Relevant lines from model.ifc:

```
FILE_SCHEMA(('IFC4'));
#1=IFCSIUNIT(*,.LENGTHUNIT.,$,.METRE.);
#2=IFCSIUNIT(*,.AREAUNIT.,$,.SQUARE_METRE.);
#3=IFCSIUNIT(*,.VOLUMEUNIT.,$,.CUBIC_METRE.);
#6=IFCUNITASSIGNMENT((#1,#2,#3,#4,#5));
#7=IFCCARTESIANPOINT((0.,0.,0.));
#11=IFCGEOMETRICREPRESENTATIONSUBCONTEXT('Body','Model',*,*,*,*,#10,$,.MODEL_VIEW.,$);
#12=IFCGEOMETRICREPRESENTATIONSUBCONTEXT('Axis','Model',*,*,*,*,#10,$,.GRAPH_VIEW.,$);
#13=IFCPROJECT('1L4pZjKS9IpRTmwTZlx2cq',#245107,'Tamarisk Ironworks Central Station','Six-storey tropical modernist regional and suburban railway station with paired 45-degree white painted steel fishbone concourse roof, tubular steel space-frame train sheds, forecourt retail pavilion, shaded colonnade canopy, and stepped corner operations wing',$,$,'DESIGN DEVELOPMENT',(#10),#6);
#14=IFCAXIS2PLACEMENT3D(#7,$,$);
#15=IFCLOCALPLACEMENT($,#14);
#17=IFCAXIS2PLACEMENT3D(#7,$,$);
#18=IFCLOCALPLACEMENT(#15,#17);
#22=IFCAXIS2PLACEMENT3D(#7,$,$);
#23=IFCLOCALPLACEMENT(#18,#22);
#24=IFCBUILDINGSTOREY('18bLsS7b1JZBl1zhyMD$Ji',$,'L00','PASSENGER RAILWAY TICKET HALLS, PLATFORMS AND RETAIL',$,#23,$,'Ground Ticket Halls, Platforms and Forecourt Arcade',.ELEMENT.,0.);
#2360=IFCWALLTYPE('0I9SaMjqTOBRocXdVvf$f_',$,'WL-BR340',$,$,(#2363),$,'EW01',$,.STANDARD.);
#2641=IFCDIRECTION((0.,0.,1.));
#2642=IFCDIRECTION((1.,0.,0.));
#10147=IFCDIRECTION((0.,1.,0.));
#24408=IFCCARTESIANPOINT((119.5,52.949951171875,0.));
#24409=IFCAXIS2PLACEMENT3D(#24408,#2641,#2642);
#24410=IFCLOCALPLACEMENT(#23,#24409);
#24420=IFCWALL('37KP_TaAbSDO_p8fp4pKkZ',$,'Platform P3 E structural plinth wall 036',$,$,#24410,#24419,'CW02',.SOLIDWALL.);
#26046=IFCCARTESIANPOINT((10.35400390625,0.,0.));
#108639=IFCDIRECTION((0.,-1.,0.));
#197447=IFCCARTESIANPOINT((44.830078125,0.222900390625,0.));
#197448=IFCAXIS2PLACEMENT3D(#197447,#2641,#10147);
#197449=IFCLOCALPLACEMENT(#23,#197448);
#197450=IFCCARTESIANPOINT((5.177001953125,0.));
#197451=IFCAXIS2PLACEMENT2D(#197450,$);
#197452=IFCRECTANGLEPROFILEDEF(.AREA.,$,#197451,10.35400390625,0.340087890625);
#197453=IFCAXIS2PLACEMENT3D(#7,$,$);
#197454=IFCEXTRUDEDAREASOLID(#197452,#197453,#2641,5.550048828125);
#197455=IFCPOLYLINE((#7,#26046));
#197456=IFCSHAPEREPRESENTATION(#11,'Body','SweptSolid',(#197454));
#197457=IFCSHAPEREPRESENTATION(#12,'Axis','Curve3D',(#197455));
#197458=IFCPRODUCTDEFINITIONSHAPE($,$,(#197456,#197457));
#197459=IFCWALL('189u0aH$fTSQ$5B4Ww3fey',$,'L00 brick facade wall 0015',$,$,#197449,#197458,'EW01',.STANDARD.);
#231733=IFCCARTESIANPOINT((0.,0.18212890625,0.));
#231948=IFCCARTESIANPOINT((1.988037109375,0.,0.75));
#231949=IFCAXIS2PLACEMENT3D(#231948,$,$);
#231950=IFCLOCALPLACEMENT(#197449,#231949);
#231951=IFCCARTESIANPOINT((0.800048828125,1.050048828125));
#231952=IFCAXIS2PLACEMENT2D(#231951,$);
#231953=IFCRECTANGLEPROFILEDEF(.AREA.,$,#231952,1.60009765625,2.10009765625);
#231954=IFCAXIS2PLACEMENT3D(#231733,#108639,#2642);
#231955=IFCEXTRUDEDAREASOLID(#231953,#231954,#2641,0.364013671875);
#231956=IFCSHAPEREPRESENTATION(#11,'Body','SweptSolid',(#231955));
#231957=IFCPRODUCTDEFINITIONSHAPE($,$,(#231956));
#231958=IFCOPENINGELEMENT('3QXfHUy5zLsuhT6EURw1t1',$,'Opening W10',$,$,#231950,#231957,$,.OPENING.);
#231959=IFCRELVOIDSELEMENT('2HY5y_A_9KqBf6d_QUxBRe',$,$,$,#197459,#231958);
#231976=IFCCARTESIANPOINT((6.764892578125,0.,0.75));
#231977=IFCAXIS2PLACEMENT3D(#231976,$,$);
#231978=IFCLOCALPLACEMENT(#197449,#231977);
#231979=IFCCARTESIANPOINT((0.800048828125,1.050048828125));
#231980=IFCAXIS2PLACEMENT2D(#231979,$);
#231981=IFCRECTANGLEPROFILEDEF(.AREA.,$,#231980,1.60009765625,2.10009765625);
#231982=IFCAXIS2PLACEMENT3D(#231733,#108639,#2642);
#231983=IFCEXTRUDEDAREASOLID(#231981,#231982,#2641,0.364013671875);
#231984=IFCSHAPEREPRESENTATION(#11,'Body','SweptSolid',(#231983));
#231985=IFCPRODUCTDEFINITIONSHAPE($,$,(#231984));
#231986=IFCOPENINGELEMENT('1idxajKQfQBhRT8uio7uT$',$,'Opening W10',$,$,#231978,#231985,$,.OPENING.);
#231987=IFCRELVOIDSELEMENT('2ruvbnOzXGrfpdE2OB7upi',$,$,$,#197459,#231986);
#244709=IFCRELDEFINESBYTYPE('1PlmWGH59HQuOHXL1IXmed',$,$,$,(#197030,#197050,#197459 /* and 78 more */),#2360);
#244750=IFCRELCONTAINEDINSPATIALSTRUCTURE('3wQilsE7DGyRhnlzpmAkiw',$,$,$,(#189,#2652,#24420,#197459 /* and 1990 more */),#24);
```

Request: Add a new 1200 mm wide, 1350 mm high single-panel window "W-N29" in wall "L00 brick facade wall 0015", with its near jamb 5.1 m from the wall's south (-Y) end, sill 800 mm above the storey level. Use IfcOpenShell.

```python
import numpy as np
import ifcopenshell
import ifcopenshell.api.feature
import ifcopenshell.api.geometry
import ifcopenshell.api.root
import ifcopenshell.api.spatial
import ifcopenshell.geom
import ifcopenshell.util.element
import ifcopenshell.util.placement
import ifcopenshell.util.representation
import ifcopenshell.util.shape
import ifcopenshell.util.unit

model = ifcopenshell.open("model.ifc")
unit_scale = ifcopenshell.util.unit.calculate_unit_scale(model)
settings = ifcopenshell.geom.settings()


def volume(element):
    """Net volume in cubic metres, openings subtracted."""
    shape = ifcopenshell.geom.create_shape(settings, element)
    return ifcopenshell.util.shape.get_volume(shape.geometry)


wall = model.by_guid("189u0aH$fTSQ$5B4Ww3fey")
storey = ifcopenshell.util.element.get_container(wall, ifc_class="IfcBuildingStorey")
context = ifcopenshell.util.representation.get_context(model, "Model", "Body", "MODEL_VIEW")
before = volume(wall)

width, height, from_end, sill = 1.2, 1.35, 5.1, 0.8  # metres

# The wall runs along its own X axis, and the end named is its -X end.
wall_shape = ifcopenshell.geom.create_shape(settings, wall)
x, y, z = ifcopenshell.util.shape.get_vertices(wall_shape.geometry).T
start = x.min() + from_end
face, thickness = float(y.min()), float(y.max() - y.min())
wall_matrix = ifcopenshell.util.placement.get_local_placement(wall.ObjectPlacement)
level = ifcopenshell.util.placement.get_local_placement(storey.ObjectPlacement)[2, 3]


def in_wall(x, y):
    """Placement at x, y metres in the wall's axes, at sill height."""
    matrix = wall_matrix.copy()
    matrix[:, 3] = wall_matrix @ np.array([x / unit_scale, y / unit_scale, 0.0, 1.0])
    matrix[2, 3] = level + sill / unit_scale
    return matrix


# Opening: a box that overshoots both wall faces by 50 mm.
opening = ifcopenshell.api.root.create_entity(model, ifc_class="IfcOpeningElement", predefined_type="OPENING")
box = ifcopenshell.api.geometry.add_wall_representation(
    model, context=context, length=width, height=height, thickness=thickness + 0.1
)
ifcopenshell.api.geometry.assign_representation(model, product=opening, representation=box)
ifcopenshell.api.geometry.edit_object_placement(model, product=opening, matrix=in_wall(start, face - 0.05), is_si=False)
ifcopenshell.api.feature.add_feature(model, feature=opening, element=wall)

window = ifcopenshell.api.root.create_entity(model, ifc_class="IfcWindow", name="W-N29", predefined_type="WINDOW")
window.OverallWidth, window.OverallHeight = width / unit_scale, height / unit_scale
window.PartitioningType = "SINGLE_PANEL"
body = ifcopenshell.api.geometry.add_window_representation(
    model,
    context=context,
    overall_width=window.OverallWidth,
    overall_height=window.OverallHeight,
    partition_type="SINGLE_PANEL",
)
ifcopenshell.api.geometry.assign_representation(model, product=window, representation=body)
ifcopenshell.api.spatial.assign_container(model, products=[window], relating_structure=storey)
ifcopenshell.api.feature.add_filling(model, opening=opening, element=window)

# Centre the window in the wall's thickness.
ifcopenshell.api.geometry.edit_object_placement(model, product=window, matrix=in_wall(start, face), is_si=False)
window_shape = ifcopenshell.geom.create_shape(settings, window)
depth = ifcopenshell.util.shape.get_vertices(window_shape.geometry)[:, 1]
offset = face + thickness / 2 - (depth.min() + depth.max()) / 2
ifcopenshell.api.geometry.edit_object_placement(model, product=window, matrix=in_wall(start, offset), is_si=False)

after = volume(wall)

print(f"wall volume {before:.3f} -> {after:.3f} m3")

model.write("model_edited.ifc")
```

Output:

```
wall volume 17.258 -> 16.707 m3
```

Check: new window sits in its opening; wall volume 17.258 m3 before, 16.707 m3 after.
